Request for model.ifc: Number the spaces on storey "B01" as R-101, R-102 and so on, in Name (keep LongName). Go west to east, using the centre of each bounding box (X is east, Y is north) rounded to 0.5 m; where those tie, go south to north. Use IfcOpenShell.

First a look at what the model holds.

```python
import ifcopenshell
import ifcopenshell.util.element
import ifcopenshell.util.placement

model = ifcopenshell.open("model.ifc")
print(model.schema)
storey = next(s for s in model.by_type("IfcBuildingStorey") if s.Name == "B01")
spaces = [e for e in ifcopenshell.util.element.get_decomposition(storey) if e.is_a("IfcSpace")]
for e in sorted(spaces, key=lambda e: e.id()):
    origin = ifcopenshell.util.placement.get_local_placement(e.ObjectPlacement)[:3, 3]
    print(e.id(), e.Name, e.LongName, origin.round(2) + 0.0, sep=" | ")
```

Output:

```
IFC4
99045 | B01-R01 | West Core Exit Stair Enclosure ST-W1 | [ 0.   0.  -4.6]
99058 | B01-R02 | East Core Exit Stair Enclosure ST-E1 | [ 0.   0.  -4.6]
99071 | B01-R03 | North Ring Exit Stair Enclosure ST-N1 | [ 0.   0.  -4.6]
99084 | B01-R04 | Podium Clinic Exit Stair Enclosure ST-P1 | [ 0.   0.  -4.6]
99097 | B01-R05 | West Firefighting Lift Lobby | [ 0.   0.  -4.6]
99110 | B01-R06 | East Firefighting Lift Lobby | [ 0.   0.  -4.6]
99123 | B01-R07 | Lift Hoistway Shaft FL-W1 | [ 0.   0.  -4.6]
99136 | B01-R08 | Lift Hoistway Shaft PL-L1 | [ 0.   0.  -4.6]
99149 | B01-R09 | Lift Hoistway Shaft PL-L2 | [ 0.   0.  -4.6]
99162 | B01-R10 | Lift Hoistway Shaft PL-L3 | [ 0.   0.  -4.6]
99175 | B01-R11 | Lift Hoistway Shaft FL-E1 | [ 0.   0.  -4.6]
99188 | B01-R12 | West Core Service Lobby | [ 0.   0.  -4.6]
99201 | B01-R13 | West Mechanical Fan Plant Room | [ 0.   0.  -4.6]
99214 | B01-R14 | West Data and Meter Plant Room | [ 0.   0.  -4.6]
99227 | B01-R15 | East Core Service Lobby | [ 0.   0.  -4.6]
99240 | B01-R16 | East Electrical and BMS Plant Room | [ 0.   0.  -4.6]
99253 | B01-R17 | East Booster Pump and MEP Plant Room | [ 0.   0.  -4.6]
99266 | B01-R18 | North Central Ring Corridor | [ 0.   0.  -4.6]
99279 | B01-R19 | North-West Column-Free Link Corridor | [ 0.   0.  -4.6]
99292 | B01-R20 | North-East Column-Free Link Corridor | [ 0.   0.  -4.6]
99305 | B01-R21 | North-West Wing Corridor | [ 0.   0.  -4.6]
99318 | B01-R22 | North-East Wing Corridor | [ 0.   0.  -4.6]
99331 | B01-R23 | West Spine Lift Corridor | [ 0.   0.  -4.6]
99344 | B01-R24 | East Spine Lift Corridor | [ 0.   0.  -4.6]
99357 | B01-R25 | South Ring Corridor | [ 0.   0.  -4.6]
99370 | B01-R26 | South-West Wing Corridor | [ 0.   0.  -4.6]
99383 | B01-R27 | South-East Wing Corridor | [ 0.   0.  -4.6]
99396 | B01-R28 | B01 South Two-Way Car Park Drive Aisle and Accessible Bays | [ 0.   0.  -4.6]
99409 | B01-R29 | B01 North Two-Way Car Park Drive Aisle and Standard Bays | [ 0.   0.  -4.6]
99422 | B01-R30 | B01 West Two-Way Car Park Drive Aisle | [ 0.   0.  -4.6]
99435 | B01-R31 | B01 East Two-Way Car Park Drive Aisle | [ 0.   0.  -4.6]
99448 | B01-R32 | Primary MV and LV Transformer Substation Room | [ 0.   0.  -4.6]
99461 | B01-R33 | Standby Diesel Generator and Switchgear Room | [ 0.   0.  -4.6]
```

```python
import ifcopenshell
import ifcopenshell.geom
import ifcopenshell.util.element
import ifcopenshell.util.shape

model = ifcopenshell.open("model.ifc")
settings = ifcopenshell.geom.settings()
settings.set("use-world-coords", True)


def centre(element):
    shape = ifcopenshell.geom.create_shape(settings, element)
    return ifcopenshell.util.shape.get_bbox_centroid(shape.geometry)


storey = next(s for s in model.by_type("IfcBuildingStorey") if s.Name == "B01")
spaces = [e for e in ifcopenshell.util.element.get_decomposition(storey) if e.is_a("IfcSpace")]

# Insertion points can sit at a corner or the storey origin, so sort by the geometry (in metres).
centres = {e: centre(e) for e in spaces}
spaces.sort(key=lambda e: (round(centres[e][0] / 0.5), centres[e][1]))

for i, e in enumerate(spaces, start=1):
    number = f"R-1{i:02d}"
    e.Name = number
    print(e.id(), number)

model.write("model_updated.ifc")
```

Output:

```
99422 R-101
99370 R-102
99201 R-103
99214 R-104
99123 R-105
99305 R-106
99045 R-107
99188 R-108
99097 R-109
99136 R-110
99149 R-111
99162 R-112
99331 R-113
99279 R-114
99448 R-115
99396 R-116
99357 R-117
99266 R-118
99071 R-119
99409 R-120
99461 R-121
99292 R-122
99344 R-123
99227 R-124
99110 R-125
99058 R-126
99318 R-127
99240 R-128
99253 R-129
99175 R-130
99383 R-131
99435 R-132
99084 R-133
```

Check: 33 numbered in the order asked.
